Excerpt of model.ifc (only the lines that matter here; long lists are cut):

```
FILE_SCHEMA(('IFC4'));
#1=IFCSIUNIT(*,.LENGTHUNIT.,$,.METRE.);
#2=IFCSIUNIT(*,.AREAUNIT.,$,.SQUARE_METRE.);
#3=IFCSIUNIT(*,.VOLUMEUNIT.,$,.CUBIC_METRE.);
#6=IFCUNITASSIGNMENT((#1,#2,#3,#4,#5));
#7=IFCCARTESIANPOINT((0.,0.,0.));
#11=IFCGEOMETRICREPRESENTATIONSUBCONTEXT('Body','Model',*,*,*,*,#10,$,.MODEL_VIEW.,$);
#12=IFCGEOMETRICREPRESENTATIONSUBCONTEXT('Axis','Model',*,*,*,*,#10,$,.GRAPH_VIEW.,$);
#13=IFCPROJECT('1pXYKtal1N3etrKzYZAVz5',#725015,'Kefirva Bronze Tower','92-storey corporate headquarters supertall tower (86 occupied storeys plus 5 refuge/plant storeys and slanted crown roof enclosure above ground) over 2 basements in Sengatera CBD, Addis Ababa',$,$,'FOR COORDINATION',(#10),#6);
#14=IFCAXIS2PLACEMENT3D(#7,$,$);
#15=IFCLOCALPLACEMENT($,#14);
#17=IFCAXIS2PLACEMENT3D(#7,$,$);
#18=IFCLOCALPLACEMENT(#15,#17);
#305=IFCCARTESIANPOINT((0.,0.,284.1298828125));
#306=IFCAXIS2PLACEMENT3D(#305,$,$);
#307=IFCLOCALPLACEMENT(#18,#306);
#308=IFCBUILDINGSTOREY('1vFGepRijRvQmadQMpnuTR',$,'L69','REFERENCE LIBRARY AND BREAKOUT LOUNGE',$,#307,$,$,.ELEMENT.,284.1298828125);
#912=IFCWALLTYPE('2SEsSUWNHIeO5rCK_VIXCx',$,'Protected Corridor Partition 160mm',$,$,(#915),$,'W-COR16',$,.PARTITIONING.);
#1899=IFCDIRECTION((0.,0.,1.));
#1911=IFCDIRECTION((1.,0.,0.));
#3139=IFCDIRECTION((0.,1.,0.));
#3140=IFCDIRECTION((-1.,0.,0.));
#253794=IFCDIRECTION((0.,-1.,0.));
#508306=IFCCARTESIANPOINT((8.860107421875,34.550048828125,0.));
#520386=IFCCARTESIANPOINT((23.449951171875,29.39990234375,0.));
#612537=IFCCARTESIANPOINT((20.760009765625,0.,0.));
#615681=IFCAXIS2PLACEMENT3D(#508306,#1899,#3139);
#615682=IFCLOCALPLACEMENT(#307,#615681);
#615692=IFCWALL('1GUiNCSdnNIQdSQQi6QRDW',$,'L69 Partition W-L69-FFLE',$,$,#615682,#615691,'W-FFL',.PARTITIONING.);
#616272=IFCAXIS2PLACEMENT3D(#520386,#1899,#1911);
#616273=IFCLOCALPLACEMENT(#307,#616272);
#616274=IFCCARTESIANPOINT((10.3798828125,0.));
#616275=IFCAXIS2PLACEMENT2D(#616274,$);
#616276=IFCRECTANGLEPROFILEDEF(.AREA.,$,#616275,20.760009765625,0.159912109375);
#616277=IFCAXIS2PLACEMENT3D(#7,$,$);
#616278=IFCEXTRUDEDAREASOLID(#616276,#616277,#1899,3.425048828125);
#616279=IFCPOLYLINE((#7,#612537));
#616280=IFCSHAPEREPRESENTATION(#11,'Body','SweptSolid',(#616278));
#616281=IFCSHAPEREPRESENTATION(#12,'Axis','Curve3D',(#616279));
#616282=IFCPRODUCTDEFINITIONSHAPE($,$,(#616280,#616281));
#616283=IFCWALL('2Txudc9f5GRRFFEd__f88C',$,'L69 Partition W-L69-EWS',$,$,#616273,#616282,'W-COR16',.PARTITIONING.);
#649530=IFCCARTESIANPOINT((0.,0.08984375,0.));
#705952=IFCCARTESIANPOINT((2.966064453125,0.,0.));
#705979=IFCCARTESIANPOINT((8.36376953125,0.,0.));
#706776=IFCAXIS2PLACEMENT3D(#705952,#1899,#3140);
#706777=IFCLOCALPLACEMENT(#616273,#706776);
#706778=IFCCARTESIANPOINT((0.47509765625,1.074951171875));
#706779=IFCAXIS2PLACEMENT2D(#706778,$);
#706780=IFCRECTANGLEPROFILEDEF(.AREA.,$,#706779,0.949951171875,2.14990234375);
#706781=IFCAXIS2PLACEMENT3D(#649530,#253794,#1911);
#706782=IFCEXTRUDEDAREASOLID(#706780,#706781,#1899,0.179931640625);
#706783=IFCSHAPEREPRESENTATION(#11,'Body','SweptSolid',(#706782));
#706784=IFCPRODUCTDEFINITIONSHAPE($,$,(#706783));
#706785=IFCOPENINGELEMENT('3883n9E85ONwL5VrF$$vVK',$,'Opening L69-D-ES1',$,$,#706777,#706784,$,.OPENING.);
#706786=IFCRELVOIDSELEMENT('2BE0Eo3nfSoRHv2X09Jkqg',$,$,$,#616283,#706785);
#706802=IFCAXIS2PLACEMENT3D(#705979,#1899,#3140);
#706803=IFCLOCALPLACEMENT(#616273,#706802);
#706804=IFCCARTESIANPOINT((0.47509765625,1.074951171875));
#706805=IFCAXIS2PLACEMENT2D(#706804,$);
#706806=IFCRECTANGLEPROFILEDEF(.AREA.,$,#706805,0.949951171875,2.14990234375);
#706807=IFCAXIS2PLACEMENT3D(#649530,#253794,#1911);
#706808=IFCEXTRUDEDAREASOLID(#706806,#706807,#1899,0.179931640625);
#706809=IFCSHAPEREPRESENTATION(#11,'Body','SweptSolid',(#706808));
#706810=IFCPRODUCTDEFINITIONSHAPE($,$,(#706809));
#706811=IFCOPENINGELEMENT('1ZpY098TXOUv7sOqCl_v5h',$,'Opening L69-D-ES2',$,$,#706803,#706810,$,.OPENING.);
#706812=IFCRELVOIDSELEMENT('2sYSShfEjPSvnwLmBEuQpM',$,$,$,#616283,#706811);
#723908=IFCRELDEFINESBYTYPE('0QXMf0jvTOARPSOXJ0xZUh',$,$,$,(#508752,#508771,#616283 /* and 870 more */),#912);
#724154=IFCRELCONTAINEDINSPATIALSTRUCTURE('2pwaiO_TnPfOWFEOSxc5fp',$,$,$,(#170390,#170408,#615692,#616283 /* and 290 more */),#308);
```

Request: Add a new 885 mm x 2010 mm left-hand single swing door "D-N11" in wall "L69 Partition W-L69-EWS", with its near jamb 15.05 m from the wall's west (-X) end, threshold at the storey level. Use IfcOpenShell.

```python
import numpy as np
import ifcopenshell
import ifcopenshell.api.feature
import ifcopenshell.api.geometry
import ifcopenshell.api.root
import ifcopenshell.api.spatial
import ifcopenshell.geom
import ifcopenshell.util.element
import ifcopenshell.util.placement
import ifcopenshell.util.representation
import ifcopenshell.util.shape
import ifcopenshell.util.unit

model = ifcopenshell.open("model.ifc")
unit_scale = ifcopenshell.util.unit.calculate_unit_scale(model)
settings = ifcopenshell.geom.settings()


def volume(element):
    """Net volume in cubic metres, openings subtracted."""
    shape = ifcopenshell.geom.create_shape(settings, element)
    return ifcopenshell.util.shape.get_volume(shape.geometry)


wall = model.by_id(616283)
storey = ifcopenshell.util.element.get_container(wall, ifc_class="IfcBuildingStorey")
context = ifcopenshell.util.representation.get_context(model, "Model", "Body", "MODEL_VIEW")
before = volume(wall)

width, height, from_end, sill = 0.885, 2.01, 15.05, 0.0  # metres

# The wall runs along its own X axis, and the end named is its -X end.
wall_shape = ifcopenshell.geom.create_shape(settings, wall)
x, y, z = ifcopenshell.util.shape.get_vertices(wall_shape.geometry).T
start = x.min() + from_end
face, thickness = float(y.min()), float(y.max() - y.min())
wall_matrix = ifcopenshell.util.placement.get_local_placement(wall.ObjectPlacement)
level = ifcopenshell.util.placement.get_local_placement(storey.ObjectPlacement)[2, 3]


def in_wall(x, y):
    """Placement at x, y metres in the wall's axes, at sill height."""
    matrix = wall_matrix.copy()
    matrix[:, 3] = wall_matrix @ np.array([x / unit_scale, y / unit_scale, 0.0, 1.0])
    matrix[2, 3] = level + sill / unit_scale
    return matrix


# Opening: a box that overshoots both wall faces by 50 mm.
opening = ifcopenshell.api.root.create_entity(model, ifc_class="IfcOpeningElement", predefined_type="OPENING")
box = ifcopenshell.api.geometry.add_wall_representation(
    model, context=context, length=width, height=height, thickness=thickness + 0.1
)
ifcopenshell.api.geometry.assign_representation(model, product=opening, representation=box)
ifcopenshell.api.geometry.edit_object_placement(model, product=opening, matrix=in_wall(start, face - 0.05), is_si=False)
ifcopenshell.api.feature.add_feature(model, feature=opening, element=wall)

door = ifcopenshell.api.root.create_entity(model, ifc_class="IfcDoor", name="D-N11", predefined_type="DOOR")
door.OverallWidth, door.OverallHeight = width / unit_scale, height / unit_scale
door.OperationType = "SINGLE_SWING_LEFT"
body = ifcopenshell.api.geometry.add_door_representation(
    model,
    context=context,
    overall_width=door.OverallWidth,
    overall_height=door.OverallHeight,
    operation_type="SINGLE_SWING_LEFT",
    lining_properties={"LiningDepth": thickness / unit_scale, "ThresholdDepth": thickness / unit_scale},
)
ifcopenshell.api.geometry.assign_representation(model, product=door, representation=body)
ifcopenshell.api.spatial.assign_container(model, products=[door], relating_structure=storey)
ifcopenshell.api.feature.add_filling(model, opening=opening, element=door)

# The lining spans the wall, so the door starts at the wall face.
ifcopenshell.api.geometry.edit_object_placement(model, product=door, matrix=in_wall(start, face), is_si=False)

after = volume(wall)

print(f"wall volume {before:.3f} -> {after:.3f} m3")

model.write("model_rev.ifc")
```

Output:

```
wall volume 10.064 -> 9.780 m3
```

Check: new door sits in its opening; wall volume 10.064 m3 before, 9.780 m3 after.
